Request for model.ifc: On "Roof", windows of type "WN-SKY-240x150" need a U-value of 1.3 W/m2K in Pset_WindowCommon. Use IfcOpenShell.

First a look at what the model holds.

```python
import ifcopenshell
import ifcopenshell.util.element

model = ifcopenshell.open("model.ifc")
print(model.schema)
storey = next(s for s in model.by_type("IfcBuildingStorey") if s.Name == "Roof")
windows = [e for e in ifcopenshell.util.element.get_decomposition(storey) if e.is_a("IfcWindow")]
seen = {}
for e in windows:
    element_type = ifcopenshell.util.element.get_type(e)
    key = (element_type.Name if element_type != e and element_type else None, ifcopenshell.util.element.get_pset(e, "Pset_WindowCommon", "ThermalTransmittance"))
    seen[key] = seen.get(key, 0) + 1
for (name, value), count in sorted(seen.items(), key=str):
    print(count, "x", name, "|", value)
```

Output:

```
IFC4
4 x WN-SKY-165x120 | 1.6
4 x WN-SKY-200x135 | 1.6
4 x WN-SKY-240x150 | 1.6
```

```python
import ifcopenshell
import ifcopenshell.api.pset
import ifcopenshell.util.element

model = ifcopenshell.open("model.ifc")

storey = next(s for s in model.by_type("IfcBuildingStorey") if s.Name == "Roof")
windows = [e for e in ifcopenshell.util.element.get_decomposition(storey) if e.is_a("IfcWindow")]

count = 0
for e in windows:
    element_type = ifcopenshell.util.element.get_type(e)
    if element_type in (None, e) or element_type.Name != "WN-SKY-240x150":
        continue
    # add_pset returns the element's existing set when there is one.
    pset = ifcopenshell.api.pset.add_pset(model, product=e, name="Pset_WindowCommon")
    ifcopenshell.api.pset.edit_pset(model, pset=pset, properties={"ThermalTransmittance": 1.3})
    count += 1

print(count, "windows updated")

model.write("model_updated.ifc")
```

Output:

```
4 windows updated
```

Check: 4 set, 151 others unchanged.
